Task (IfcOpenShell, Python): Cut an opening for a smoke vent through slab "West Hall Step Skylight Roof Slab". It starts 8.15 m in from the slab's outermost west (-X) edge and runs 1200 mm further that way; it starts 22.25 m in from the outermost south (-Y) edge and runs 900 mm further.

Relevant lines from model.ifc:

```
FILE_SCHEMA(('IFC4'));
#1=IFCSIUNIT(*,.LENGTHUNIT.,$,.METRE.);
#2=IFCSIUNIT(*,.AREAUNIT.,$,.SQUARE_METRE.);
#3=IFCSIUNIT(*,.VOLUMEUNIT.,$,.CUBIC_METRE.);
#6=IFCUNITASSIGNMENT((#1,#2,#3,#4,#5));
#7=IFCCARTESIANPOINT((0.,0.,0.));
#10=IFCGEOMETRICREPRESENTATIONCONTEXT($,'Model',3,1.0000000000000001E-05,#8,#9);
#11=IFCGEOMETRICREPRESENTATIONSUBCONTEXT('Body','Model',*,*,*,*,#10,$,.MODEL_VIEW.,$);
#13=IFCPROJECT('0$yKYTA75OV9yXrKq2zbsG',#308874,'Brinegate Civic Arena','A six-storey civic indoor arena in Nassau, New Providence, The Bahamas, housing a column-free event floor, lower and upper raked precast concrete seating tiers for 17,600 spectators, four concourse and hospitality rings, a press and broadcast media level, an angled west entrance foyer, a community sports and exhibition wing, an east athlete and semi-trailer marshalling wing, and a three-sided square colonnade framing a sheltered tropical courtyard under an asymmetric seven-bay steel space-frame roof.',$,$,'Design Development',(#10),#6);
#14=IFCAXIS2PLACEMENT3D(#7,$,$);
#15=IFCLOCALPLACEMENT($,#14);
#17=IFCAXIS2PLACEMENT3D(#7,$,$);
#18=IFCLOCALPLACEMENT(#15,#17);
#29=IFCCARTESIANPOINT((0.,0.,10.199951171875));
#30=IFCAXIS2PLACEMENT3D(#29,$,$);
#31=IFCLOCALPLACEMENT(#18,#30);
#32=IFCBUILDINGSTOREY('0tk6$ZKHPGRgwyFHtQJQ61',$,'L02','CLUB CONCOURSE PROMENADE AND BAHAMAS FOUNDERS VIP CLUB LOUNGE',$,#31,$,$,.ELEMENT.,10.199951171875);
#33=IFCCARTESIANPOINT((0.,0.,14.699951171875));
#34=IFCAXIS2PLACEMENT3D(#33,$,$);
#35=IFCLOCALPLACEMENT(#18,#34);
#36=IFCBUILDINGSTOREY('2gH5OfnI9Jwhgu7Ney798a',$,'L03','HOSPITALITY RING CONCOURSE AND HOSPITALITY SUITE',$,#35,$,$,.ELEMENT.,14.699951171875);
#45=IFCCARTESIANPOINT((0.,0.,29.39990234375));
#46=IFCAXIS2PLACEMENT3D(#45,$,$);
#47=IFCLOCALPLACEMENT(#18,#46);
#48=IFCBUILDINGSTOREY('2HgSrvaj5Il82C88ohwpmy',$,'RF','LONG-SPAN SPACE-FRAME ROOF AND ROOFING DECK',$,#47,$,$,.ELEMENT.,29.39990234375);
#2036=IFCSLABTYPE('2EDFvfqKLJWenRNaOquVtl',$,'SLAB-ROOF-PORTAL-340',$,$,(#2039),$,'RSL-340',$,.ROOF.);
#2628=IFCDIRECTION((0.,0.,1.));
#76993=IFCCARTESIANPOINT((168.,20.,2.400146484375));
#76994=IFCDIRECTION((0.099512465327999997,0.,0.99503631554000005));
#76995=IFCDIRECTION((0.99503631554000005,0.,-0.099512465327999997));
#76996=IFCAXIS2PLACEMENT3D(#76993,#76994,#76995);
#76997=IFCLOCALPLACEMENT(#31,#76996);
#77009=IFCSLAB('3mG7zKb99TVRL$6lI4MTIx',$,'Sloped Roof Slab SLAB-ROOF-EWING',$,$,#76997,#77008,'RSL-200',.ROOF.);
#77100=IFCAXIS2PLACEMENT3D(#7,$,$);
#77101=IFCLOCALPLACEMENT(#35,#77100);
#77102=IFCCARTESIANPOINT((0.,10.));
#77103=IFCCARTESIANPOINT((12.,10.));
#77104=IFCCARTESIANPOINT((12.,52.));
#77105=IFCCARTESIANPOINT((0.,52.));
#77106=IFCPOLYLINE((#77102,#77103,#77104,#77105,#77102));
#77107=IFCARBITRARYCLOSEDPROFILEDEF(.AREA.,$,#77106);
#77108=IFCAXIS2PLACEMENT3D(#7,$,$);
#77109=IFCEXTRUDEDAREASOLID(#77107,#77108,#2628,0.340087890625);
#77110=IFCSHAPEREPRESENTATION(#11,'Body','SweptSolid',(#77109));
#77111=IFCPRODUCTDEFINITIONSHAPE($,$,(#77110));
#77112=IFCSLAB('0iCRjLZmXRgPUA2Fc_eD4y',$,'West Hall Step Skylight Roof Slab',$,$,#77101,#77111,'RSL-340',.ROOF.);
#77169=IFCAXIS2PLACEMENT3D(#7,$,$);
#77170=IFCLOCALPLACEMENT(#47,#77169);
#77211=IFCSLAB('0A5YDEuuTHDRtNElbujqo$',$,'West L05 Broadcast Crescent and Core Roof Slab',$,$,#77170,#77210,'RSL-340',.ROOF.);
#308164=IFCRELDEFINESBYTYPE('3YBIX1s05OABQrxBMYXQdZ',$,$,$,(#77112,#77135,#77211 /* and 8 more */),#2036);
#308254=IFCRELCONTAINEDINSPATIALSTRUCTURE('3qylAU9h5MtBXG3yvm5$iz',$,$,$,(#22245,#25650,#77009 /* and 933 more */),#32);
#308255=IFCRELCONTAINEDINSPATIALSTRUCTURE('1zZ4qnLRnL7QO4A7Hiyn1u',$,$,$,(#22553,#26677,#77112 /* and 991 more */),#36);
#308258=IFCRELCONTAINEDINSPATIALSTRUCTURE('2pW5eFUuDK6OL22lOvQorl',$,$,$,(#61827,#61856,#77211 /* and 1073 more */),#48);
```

```python
import numpy as np
import ifcopenshell
import ifcopenshell.api.feature
import ifcopenshell.api.geometry
import ifcopenshell.api.root
import ifcopenshell.geom
import ifcopenshell.util.placement
import ifcopenshell.util.representation
import ifcopenshell.util.shape
import ifcopenshell.util.unit

model = ifcopenshell.open("model.ifc")
unit_scale = ifcopenshell.util.unit.calculate_unit_scale(model)
settings = ifcopenshell.geom.settings()


def volume(element):
    """Net volume in cubic metres, openings subtracted."""
    shape = ifcopenshell.geom.create_shape(settings, element)
    return ifcopenshell.util.shape.get_volume(shape.geometry)


slab = model.by_id(77112)
before = volume(slab)

# Extent in the slab's own axes, in metres. The edges named are its -X and -Y sides.
slab_shape = ifcopenshell.geom.create_shape(settings, slab)
vertices = ifcopenshell.util.shape.get_vertices(slab_shape.geometry)
x_min, y_min, bottom = vertices.min(axis=0)
top = vertices[:, 2].max()

opening = ifcopenshell.api.root.create_entity(model, ifc_class="IfcOpeningElement", name="Smoke vent opening", predefined_type="OPENING")
context = ifcopenshell.util.representation.get_context(model, "Model", "Body", "MODEL_VIEW")
width, depth = 1.2, 0.9
outline = [(0.0, 0.0), (width, 0.0), (width, depth), (0.0, depth), (0.0, 0.0)]
# Overshoot both faces by 50 mm so the cut is clean.
shape = ifcopenshell.api.geometry.add_slab_representation(
    model, context=context, depth=top - bottom + 0.1, polyline=outline
)
ifcopenshell.api.geometry.assign_representation(model, product=opening, representation=shape)

matrix = ifcopenshell.util.placement.get_local_placement(slab.ObjectPlacement)
matrix[:, 3] = matrix @ np.append(np.array([x_min + 8.15, y_min + 22.25, bottom - 0.05]) / unit_scale, 1.0)
ifcopenshell.api.geometry.edit_object_placement(model, product=opening, matrix=matrix, is_si=False)
ifcopenshell.api.feature.add_feature(model, feature=opening, element=slab)

after = volume(slab)

print(f"slab volume {before:.3f} -> {after:.3f} m3")

model.write("model_updated.ifc")
```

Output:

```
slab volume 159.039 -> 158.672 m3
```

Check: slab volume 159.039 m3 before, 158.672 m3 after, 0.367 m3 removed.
